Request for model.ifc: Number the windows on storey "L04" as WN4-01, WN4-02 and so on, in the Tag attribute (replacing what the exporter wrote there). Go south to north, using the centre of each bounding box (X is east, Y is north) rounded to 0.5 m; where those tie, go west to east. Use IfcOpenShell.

First a look at what the model holds.

```python
import ifcopenshell
import ifcopenshell.util.element
import ifcopenshell.util.placement

model = ifcopenshell.open("model.ifc")
print(model.schema)
storey = next(s for s in model.by_type("IfcBuildingStorey") if s.Name == "L04")
windows = [e for e in ifcopenshell.util.element.get_decomposition(storey) if e.is_a("IfcWindow")]
for e in sorted(windows, key=lambda e: e.id()):
    origin = ifcopenshell.util.placement.get_local_placement(e.ObjectPlacement)[:3, 3]
    print(e.id(), e.Tag, e.Name, origin.round(2) + 0.0, sep=" | ")
```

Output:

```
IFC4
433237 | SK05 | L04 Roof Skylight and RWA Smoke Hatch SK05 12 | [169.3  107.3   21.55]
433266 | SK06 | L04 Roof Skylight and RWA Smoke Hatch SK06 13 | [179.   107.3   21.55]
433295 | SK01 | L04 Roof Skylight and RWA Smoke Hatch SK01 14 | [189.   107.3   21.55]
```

```python
import ifcopenshell
import ifcopenshell.geom
import ifcopenshell.util.element
import ifcopenshell.util.shape

model = ifcopenshell.open("model.ifc")
settings = ifcopenshell.geom.settings()
settings.set("use-world-coords", True)


def centre(element):
    shape = ifcopenshell.geom.create_shape(settings, element)
    return ifcopenshell.util.shape.get_bbox_centroid(shape.geometry)


storey = next(s for s in model.by_type("IfcBuildingStorey") if s.Name == "L04")
windows = [e for e in ifcopenshell.util.element.get_decomposition(storey) if e.is_a("IfcWindow")]

# Insertion points can sit at a corner or the storey origin, so sort by the geometry (in metres).
centres = {e: centre(e) for e in windows}
windows.sort(key=lambda e: (round(centres[e][1] / 0.5), centres[e][0]))

for i, e in enumerate(windows, start=1):
    number = f"WN4-{i:02d}"
    e.Tag = number
    print(e.id(), number)

model.write("model_edited.ifc")
```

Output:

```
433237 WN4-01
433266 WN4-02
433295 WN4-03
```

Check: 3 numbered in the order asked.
